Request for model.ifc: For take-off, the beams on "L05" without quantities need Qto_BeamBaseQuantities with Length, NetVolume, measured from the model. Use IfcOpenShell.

First a look at what the model holds.

```python
import ifcopenshell
import ifcopenshell.util.element
import ifcopenshell.util.unit

model = ifcopenshell.open("model.ifc")
print(model.schema)
for unit_type in ("LENGTHUNIT", "AREAUNIT", "VOLUMEUNIT"):
    print(unit_type, ifcopenshell.util.unit.calculate_unit_scale(model, unit_type))
storey = next(s for s in model.by_type("IfcBuildingStorey") if s.Name == "L05")
beams = [e for e in ifcopenshell.util.element.get_decomposition(storey) if e.is_a("IfcBeam")]
for e in sorted(beams, key=lambda e: e.id()):
    print(e.id(), e.is_a(), e.Name, list(ifcopenshell.util.element.get_psets(e, qtos_only=True)), sep=" | ")
```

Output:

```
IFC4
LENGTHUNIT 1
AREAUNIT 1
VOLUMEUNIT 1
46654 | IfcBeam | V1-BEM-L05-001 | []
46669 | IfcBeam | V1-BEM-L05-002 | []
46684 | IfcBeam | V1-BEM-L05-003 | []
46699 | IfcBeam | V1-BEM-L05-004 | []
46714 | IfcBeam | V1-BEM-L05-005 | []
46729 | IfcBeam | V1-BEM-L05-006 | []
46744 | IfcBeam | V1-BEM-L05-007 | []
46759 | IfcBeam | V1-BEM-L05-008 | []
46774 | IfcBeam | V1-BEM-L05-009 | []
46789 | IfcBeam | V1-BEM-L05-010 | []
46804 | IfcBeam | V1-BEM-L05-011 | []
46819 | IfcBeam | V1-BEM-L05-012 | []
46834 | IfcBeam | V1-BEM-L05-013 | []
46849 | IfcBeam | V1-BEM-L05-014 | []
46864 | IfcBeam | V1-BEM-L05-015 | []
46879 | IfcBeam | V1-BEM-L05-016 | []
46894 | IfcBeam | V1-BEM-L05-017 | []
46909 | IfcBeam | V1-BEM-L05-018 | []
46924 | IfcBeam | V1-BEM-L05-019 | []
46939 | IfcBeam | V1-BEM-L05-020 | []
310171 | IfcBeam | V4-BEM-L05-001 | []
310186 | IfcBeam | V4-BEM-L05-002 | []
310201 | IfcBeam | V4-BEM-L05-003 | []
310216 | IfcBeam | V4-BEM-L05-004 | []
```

```python
import ifcopenshell
import ifcopenshell.api.pset
import ifcopenshell.geom
import ifcopenshell.util.element
import ifcopenshell.util.shape
import ifcopenshell.util.unit

model = ifcopenshell.open("model.ifc")
unit_scale = ifcopenshell.util.unit.calculate_unit_scale(model)
volume_scale = ifcopenshell.util.unit.calculate_unit_scale(model, "VOLUMEUNIT")
settings = ifcopenshell.geom.settings()

storey = next(s for s in model.by_type("IfcBuildingStorey") if s.Name == "L05")
beams = [e for e in ifcopenshell.util.element.get_decomposition(storey) if e.is_a("IfcBeam")]

for e in sorted(beams, key=lambda e: e.id()):
    if ifcopenshell.util.element.get_psets(e, qtos_only=True, should_inherit=False):
        continue
    # Geometry comes back in metres, in the element's own axes.
    shape = ifcopenshell.geom.create_shape(settings, e)
    values = {
        "Length": ifcopenshell.util.shape.get_max_xyz(shape.geometry) / unit_scale,
        "NetVolume": ifcopenshell.util.shape.get_volume(shape.geometry) / volume_scale,
    }
    qto = ifcopenshell.api.pset.add_qto(model, product=e, name="Qto_BeamBaseQuantities")
    ifcopenshell.api.pset.edit_qto(model, qto=qto, properties=values)
    print(e.id(), {k: round(v, 3) for k, v in values.items()})

model.write("model_v2.ifc")
```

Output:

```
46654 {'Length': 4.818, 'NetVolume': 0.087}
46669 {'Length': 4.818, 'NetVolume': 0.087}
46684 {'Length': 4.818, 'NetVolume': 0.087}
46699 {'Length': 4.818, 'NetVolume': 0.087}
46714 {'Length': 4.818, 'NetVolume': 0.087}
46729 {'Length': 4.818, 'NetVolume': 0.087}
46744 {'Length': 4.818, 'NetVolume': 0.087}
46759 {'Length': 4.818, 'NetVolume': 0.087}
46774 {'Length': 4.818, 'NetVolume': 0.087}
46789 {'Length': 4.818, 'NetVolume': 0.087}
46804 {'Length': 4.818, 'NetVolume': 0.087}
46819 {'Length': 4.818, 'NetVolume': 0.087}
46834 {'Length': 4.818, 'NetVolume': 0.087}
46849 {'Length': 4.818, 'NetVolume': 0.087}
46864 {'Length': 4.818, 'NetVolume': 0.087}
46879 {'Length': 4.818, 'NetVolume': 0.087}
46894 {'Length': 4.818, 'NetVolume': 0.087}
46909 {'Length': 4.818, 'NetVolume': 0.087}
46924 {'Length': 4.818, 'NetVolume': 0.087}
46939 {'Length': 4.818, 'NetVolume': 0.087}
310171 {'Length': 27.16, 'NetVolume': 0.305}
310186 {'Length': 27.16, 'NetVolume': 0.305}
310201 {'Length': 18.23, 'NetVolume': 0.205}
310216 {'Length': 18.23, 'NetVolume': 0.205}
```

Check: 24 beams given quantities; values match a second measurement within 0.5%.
